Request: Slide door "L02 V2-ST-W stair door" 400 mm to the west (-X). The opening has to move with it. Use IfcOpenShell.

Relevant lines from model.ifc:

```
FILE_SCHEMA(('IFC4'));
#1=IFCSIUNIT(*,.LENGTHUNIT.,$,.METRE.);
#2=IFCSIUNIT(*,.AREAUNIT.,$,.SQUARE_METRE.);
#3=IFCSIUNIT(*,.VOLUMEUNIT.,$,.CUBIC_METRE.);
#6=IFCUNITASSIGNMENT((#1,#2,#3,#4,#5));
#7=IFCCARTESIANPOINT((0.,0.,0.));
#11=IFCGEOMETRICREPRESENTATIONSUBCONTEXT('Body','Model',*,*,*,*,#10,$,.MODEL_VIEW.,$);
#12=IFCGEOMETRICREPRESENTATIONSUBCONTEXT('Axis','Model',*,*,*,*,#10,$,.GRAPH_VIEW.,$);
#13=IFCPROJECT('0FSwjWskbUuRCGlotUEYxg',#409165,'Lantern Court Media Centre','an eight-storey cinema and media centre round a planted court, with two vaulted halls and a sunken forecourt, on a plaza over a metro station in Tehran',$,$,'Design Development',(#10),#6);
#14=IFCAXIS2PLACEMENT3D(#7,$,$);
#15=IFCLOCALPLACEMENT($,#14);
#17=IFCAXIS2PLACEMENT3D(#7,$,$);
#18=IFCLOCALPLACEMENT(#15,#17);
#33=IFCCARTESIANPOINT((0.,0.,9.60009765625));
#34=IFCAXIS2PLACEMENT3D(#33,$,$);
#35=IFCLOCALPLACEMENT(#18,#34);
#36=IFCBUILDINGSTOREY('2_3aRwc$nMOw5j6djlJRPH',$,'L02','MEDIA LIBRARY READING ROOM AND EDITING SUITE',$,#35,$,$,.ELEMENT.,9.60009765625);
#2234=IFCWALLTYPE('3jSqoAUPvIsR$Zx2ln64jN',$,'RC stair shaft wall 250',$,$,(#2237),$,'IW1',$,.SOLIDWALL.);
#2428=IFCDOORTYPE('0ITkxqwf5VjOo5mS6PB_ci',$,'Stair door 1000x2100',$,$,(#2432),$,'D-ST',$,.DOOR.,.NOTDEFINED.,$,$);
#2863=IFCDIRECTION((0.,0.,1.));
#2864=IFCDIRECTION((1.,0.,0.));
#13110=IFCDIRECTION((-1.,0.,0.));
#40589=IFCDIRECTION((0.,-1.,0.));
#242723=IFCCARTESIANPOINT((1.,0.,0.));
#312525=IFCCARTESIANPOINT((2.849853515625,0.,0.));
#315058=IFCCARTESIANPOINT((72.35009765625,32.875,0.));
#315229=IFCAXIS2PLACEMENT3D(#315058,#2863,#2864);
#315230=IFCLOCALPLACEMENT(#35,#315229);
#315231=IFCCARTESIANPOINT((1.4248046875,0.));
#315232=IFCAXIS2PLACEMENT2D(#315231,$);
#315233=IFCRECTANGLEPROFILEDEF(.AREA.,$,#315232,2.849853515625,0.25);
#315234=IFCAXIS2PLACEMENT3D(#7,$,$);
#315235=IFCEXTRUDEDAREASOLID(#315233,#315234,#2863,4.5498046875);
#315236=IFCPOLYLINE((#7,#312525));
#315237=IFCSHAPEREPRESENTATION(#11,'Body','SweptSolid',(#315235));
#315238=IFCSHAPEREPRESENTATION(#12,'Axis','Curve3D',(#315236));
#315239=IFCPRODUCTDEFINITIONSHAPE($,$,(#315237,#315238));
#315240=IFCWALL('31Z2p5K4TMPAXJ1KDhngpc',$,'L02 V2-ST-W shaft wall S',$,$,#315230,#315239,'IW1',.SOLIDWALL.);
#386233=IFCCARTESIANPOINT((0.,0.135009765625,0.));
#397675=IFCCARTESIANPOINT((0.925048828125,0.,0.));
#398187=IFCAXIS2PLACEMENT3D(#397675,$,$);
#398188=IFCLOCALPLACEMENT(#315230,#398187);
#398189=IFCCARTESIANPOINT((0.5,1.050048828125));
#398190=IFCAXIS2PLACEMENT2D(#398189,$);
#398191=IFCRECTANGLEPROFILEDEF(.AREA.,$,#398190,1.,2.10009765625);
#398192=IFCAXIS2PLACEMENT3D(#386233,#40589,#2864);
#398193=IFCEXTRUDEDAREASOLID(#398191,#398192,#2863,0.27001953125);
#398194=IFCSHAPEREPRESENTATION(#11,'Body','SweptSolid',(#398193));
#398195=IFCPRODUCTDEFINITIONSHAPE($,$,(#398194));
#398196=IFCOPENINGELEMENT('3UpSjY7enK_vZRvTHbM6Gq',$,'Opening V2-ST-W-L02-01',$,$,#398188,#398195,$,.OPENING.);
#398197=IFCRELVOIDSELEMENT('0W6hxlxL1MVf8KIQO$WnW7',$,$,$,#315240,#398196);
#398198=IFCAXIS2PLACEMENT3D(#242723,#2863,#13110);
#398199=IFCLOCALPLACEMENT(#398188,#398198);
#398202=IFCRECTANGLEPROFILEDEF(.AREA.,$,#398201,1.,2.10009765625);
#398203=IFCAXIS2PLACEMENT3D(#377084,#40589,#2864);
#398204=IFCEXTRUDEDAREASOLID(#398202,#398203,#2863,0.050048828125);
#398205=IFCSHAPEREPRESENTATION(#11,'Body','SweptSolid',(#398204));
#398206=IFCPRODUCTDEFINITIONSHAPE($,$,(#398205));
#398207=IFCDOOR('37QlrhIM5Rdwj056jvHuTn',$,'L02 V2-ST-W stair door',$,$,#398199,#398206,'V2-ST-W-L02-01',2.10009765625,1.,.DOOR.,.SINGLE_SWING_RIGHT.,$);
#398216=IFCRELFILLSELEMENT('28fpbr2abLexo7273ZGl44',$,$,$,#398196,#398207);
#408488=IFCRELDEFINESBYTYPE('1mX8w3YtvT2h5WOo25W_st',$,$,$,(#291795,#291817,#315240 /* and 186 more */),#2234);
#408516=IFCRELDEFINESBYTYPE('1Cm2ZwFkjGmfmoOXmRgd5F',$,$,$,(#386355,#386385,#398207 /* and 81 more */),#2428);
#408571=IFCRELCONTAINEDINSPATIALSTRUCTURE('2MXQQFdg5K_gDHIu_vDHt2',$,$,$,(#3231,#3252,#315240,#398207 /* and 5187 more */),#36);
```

```python
import ifcopenshell
import ifcopenshell.api.geometry
import ifcopenshell.util.placement
import ifcopenshell.util.unit

model = ifcopenshell.open("model.ifc")
unit_scale = ifcopenshell.util.unit.calculate_unit_scale(model)

door = model.by_id(398207)
opening = door.FillsVoids[0].RelatingOpeningElement
wall = opening.VoidsElements[0].RelatingBuildingElement

wall_matrix = ifcopenshell.util.placement.get_local_placement(wall.ObjectPlacement)
shift = wall_matrix[:3, 0] * -0.4 / unit_scale
before = ifcopenshell.util.placement.get_local_placement(door.ObjectPlacement)[:3, 3].copy()

# The door is placed relative to its opening, so it follows when the opening moves.
matrix = ifcopenshell.util.placement.get_local_placement(opening.ObjectPlacement)
matrix[:3, 3] += shift
ifcopenshell.api.geometry.edit_object_placement(
    model, product=opening, matrix=matrix, is_si=False, should_transform_children=True
)

after = ifcopenshell.util.placement.get_local_placement(door.ObjectPlacement)[:3, 3]
print("door moved by", (after - before).round(3) + 0.0)

model.write("model_edited.ifc")
```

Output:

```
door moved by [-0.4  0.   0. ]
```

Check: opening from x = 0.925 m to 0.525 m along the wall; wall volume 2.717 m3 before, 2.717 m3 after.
